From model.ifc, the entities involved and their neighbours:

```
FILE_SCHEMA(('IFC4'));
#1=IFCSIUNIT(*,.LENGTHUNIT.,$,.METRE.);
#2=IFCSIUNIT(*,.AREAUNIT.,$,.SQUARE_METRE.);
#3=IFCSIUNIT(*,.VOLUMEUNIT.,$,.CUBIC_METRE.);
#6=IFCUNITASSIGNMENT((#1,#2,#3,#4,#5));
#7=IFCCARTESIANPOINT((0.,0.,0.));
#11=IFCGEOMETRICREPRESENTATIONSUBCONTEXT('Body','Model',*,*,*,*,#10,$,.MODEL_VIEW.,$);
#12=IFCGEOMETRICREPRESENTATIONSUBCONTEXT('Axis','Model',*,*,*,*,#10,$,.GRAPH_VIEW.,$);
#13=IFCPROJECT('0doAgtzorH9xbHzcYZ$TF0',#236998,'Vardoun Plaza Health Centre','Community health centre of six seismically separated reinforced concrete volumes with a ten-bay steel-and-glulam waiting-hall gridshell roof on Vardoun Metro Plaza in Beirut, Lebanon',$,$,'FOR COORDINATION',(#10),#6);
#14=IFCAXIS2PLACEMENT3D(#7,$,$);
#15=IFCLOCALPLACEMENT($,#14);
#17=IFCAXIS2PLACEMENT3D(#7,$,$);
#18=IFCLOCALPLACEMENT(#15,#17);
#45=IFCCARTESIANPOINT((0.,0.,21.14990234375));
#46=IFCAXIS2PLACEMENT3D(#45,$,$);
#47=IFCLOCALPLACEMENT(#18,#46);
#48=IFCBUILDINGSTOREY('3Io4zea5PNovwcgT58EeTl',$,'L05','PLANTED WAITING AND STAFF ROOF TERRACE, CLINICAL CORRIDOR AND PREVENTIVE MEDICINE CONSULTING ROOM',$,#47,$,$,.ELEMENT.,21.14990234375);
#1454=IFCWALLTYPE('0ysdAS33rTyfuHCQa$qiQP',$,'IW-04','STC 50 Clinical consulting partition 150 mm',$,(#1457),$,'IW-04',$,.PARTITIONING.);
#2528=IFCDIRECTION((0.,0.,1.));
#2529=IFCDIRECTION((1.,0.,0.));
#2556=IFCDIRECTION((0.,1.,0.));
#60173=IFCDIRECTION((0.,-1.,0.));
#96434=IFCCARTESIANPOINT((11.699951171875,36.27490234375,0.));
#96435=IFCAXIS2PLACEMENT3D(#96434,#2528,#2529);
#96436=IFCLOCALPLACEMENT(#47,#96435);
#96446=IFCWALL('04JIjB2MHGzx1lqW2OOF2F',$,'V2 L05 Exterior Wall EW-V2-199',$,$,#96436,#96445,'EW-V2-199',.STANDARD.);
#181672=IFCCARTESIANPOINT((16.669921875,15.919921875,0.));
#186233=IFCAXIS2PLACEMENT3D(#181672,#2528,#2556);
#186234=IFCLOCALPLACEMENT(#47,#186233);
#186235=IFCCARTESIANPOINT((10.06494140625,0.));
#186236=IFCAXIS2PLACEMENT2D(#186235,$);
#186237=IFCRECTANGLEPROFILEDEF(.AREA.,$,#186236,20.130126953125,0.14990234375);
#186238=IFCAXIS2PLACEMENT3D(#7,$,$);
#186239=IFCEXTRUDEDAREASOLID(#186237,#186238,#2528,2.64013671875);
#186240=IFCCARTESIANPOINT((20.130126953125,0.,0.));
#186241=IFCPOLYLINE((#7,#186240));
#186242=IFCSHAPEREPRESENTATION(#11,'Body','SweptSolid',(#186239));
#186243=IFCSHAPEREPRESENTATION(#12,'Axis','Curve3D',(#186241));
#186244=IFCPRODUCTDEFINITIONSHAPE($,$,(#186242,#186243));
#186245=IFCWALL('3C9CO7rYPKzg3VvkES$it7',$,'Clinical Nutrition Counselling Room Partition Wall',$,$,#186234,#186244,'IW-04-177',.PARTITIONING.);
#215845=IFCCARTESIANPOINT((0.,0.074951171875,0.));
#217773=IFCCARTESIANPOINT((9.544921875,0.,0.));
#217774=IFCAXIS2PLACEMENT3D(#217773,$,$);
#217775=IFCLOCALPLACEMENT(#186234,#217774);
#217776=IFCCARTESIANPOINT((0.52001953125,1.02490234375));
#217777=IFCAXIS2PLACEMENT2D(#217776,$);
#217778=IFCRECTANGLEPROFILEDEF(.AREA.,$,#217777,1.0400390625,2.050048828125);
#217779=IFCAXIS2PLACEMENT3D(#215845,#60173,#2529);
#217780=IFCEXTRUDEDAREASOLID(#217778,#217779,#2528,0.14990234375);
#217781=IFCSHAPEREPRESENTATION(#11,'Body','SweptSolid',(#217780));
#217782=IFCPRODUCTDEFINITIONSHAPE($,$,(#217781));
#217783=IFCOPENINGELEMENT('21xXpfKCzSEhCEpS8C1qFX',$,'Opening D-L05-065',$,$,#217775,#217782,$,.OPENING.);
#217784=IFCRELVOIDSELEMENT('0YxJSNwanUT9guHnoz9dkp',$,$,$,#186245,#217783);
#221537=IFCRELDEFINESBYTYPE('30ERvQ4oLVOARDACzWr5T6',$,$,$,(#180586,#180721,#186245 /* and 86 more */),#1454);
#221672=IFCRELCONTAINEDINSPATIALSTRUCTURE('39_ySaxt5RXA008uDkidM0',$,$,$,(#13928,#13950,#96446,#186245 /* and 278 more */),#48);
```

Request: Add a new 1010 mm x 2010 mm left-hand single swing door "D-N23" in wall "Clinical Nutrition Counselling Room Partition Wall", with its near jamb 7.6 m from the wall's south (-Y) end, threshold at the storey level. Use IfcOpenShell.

```python
import numpy as np
import ifcopenshell
import ifcopenshell.api.feature
import ifcopenshell.api.geometry
import ifcopenshell.api.root
import ifcopenshell.api.spatial
import ifcopenshell.geom
import ifcopenshell.util.element
import ifcopenshell.util.placement
import ifcopenshell.util.representation
import ifcopenshell.util.shape
import ifcopenshell.util.unit

model = ifcopenshell.open("model.ifc")
unit_scale = ifcopenshell.util.unit.calculate_unit_scale(model)
settings = ifcopenshell.geom.settings()


def volume(element):
    """Net volume in cubic metres, openings subtracted."""
    shape = ifcopenshell.geom.create_shape(settings, element)
    return ifcopenshell.util.shape.get_volume(shape.geometry)


wall = model.by_guid("3C9CO7rYPKzg3VvkES$it7")
storey = ifcopenshell.util.element.get_container(wall, ifc_class="IfcBuildingStorey")
context = ifcopenshell.util.representation.get_context(model, "Model", "Body", "MODEL_VIEW")
before = volume(wall)

width, height, from_end, sill = 1.01, 2.01, 7.6, 0.0  # metres

# The wall runs along its own X axis, and the end named is its -X end.
wall_shape = ifcopenshell.geom.create_shape(settings, wall)
x, y, z = ifcopenshell.util.shape.get_vertices(wall_shape.geometry).T
start = x.min() + from_end
face, thickness = float(y.min()), float(y.max() - y.min())
wall_matrix = ifcopenshell.util.placement.get_local_placement(wall.ObjectPlacement)
level = ifcopenshell.util.placement.get_local_placement(storey.ObjectPlacement)[2, 3]


def in_wall(x, y):
    """Placement at x, y metres in the wall's axes, at sill height."""
    matrix = wall_matrix.copy()
    matrix[:, 3] = wall_matrix @ np.array([x / unit_scale, y / unit_scale, 0.0, 1.0])
    matrix[2, 3] = level + sill / unit_scale
    return matrix


# Opening: a box that overshoots both wall faces by 50 mm.
opening = ifcopenshell.api.root.create_entity(model, ifc_class="IfcOpeningElement", predefined_type="OPENING")
box = ifcopenshell.api.geometry.add_wall_representation(
    model, context=context, length=width, height=height, thickness=thickness + 0.1
)
ifcopenshell.api.geometry.assign_representation(model, product=opening, representation=box)
ifcopenshell.api.geometry.edit_object_placement(model, product=opening, matrix=in_wall(start, face - 0.05), is_si=False)
ifcopenshell.api.feature.add_feature(model, feature=opening, element=wall)

door = ifcopenshell.api.root.create_entity(model, ifc_class="IfcDoor", name="D-N23", predefined_type="DOOR")
door.OverallWidth, door.OverallHeight = width / unit_scale, height / unit_scale
door.OperationType = "SINGLE_SWING_LEFT"
body = ifcopenshell.api.geometry.add_door_representation(
    model,
    context=context,
    overall_width=door.OverallWidth,
    overall_height=door.OverallHeight,
    operation_type="SINGLE_SWING_LEFT",
    lining_properties={"LiningDepth": thickness / unit_scale, "ThresholdDepth": thickness / unit_scale},
)
ifcopenshell.api.geometry.assign_representation(model, product=door, representation=body)
ifcopenshell.api.spatial.assign_container(model, products=[door], relating_structure=storey)
ifcopenshell.api.feature.add_filling(model, opening=opening, element=door)

# The lining spans the wall, so the door starts at the wall face.
ifcopenshell.api.geometry.edit_object_placement(model, product=door, matrix=in_wall(start, face), is_si=False)

after = volume(wall)

print(f"wall volume {before:.3f} -> {after:.3f} m3")

model.write("model-out.ifc")
```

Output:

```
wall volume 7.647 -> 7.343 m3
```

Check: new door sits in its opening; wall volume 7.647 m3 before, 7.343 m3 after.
